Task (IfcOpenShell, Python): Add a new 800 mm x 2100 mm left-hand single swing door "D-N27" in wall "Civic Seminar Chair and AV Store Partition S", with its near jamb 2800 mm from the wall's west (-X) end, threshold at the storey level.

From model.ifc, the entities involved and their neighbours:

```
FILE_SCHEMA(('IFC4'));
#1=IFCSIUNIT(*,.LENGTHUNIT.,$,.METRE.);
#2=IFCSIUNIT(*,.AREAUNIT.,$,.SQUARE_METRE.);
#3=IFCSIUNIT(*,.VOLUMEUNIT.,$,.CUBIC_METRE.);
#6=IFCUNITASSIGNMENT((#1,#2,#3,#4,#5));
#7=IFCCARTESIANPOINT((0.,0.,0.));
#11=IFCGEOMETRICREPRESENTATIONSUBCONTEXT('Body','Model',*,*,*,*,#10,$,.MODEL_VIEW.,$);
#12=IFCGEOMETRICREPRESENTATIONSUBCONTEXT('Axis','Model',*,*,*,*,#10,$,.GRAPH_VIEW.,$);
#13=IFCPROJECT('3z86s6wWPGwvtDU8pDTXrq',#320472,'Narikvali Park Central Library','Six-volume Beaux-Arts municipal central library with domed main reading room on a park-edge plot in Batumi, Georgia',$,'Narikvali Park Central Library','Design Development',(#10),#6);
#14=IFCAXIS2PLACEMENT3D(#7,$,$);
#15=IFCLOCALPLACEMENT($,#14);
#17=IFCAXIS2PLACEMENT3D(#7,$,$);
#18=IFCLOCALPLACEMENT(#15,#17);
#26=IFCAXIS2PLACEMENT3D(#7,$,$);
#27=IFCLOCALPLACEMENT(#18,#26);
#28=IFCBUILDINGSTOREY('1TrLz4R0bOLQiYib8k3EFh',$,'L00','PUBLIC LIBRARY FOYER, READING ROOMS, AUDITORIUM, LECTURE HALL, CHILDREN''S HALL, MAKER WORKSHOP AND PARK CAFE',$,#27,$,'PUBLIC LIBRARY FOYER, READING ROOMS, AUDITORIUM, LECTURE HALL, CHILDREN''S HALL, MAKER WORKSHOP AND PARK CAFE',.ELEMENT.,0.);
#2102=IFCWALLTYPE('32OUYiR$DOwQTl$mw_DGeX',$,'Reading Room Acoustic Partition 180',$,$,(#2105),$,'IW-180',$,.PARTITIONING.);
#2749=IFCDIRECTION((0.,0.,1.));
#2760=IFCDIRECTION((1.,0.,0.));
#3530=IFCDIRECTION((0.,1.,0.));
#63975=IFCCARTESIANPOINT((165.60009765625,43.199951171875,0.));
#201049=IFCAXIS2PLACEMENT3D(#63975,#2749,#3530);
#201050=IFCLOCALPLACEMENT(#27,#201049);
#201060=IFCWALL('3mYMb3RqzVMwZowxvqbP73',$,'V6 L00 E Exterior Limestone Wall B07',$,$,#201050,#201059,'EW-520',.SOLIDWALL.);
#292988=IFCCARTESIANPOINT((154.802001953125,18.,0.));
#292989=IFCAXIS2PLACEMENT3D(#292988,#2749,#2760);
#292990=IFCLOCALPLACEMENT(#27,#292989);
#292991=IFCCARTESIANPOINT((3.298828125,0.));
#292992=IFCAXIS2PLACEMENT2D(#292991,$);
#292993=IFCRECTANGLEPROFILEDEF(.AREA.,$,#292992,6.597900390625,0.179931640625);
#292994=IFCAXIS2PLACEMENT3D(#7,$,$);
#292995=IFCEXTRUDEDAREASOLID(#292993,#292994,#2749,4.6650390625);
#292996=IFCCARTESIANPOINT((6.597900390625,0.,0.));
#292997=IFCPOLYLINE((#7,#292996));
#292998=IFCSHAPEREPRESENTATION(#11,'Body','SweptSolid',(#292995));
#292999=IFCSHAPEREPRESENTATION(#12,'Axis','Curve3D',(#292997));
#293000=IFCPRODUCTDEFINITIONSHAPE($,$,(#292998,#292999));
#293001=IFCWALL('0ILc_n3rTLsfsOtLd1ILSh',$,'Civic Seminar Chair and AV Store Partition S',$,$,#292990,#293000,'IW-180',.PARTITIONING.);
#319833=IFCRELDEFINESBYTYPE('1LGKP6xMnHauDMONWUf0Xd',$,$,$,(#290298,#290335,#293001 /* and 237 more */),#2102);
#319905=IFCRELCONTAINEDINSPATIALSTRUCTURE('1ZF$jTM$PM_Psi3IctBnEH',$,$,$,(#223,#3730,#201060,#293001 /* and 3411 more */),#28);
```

```python
import numpy as np
import ifcopenshell
import ifcopenshell.api.feature
import ifcopenshell.api.geometry
import ifcopenshell.api.root
import ifcopenshell.api.spatial
import ifcopenshell.geom
import ifcopenshell.util.element
import ifcopenshell.util.placement
import ifcopenshell.util.representation
import ifcopenshell.util.shape
import ifcopenshell.util.unit

model = ifcopenshell.open("model.ifc")
unit_scale = ifcopenshell.util.unit.calculate_unit_scale(model)
settings = ifcopenshell.geom.settings()


def volume(element):
    """Net volume in cubic metres, openings subtracted."""
    shape = ifcopenshell.geom.create_shape(settings, element)
    return ifcopenshell.util.shape.get_volume(shape.geometry)


wall = model.by_guid("0ILc_n3rTLsfsOtLd1ILSh")
storey = ifcopenshell.util.element.get_container(wall, ifc_class="IfcBuildingStorey")
context = ifcopenshell.util.representation.get_context(model, "Model", "Body", "MODEL_VIEW")
before = volume(wall)

width, height, from_end, sill = 0.8, 2.1, 2.8, 0.0  # metres

# The wall runs along its own X axis, and the end named is its -X end.
wall_shape = ifcopenshell.geom.create_shape(settings, wall)
x, y, z = ifcopenshell.util.shape.get_vertices(wall_shape.geometry).T
start = x.min() + from_end
face, thickness = float(y.min()), float(y.max() - y.min())
wall_matrix = ifcopenshell.util.placement.get_local_placement(wall.ObjectPlacement)
level = ifcopenshell.util.placement.get_local_placement(storey.ObjectPlacement)[2, 3]


def in_wall(x, y):
    """Placement at x, y metres in the wall's axes, at sill height."""
    matrix = wall_matrix.copy()
    matrix[:, 3] = wall_matrix @ np.array([x / unit_scale, y / unit_scale, 0.0, 1.0])
    matrix[2, 3] = level + sill / unit_scale
    return matrix


# Opening: a box that overshoots both wall faces by 50 mm.
opening = ifcopenshell.api.root.create_entity(model, ifc_class="IfcOpeningElement", predefined_type="OPENING")
box = ifcopenshell.api.geometry.add_wall_representation(
    model, context=context, length=width, height=height, thickness=thickness + 0.1
)
ifcopenshell.api.geometry.assign_representation(model, product=opening, representation=box)
ifcopenshell.api.geometry.edit_object_placement(model, product=opening, matrix=in_wall(start, face - 0.05), is_si=False)
ifcopenshell.api.feature.add_feature(model, feature=opening, element=wall)

door = ifcopenshell.api.root.create_entity(model, ifc_class="IfcDoor", name="D-N27", predefined_type="DOOR")
door.OverallWidth, door.OverallHeight = width / unit_scale, height / unit_scale
door.OperationType = "SINGLE_SWING_LEFT"
body = ifcopenshell.api.geometry.add_door_representation(
    model,
    context=context,
    overall_width=door.OverallWidth,
    overall_height=door.OverallHeight,
    operation_type="SINGLE_SWING_LEFT",
    lining_properties={"LiningDepth": thickness / unit_scale, "ThresholdDepth": thickness / unit_scale},
)
ifcopenshell.api.geometry.assign_representation(model, product=door, representation=body)
ifcopenshell.api.spatial.assign_container(model, products=[door], relating_structure=storey)
ifcopenshell.api.feature.add_filling(model, opening=opening, element=door)

# The lining spans the wall, so the door starts at the wall face.
ifcopenshell.api.geometry.edit_object_placement(model, product=door, matrix=in_wall(start, face), is_si=False)

after = volume(wall)

print(f"wall volume {before:.3f} -> {after:.3f} m3")

model.write("model_edited.ifc")
```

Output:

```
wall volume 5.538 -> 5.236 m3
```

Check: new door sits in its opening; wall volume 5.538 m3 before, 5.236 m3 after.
